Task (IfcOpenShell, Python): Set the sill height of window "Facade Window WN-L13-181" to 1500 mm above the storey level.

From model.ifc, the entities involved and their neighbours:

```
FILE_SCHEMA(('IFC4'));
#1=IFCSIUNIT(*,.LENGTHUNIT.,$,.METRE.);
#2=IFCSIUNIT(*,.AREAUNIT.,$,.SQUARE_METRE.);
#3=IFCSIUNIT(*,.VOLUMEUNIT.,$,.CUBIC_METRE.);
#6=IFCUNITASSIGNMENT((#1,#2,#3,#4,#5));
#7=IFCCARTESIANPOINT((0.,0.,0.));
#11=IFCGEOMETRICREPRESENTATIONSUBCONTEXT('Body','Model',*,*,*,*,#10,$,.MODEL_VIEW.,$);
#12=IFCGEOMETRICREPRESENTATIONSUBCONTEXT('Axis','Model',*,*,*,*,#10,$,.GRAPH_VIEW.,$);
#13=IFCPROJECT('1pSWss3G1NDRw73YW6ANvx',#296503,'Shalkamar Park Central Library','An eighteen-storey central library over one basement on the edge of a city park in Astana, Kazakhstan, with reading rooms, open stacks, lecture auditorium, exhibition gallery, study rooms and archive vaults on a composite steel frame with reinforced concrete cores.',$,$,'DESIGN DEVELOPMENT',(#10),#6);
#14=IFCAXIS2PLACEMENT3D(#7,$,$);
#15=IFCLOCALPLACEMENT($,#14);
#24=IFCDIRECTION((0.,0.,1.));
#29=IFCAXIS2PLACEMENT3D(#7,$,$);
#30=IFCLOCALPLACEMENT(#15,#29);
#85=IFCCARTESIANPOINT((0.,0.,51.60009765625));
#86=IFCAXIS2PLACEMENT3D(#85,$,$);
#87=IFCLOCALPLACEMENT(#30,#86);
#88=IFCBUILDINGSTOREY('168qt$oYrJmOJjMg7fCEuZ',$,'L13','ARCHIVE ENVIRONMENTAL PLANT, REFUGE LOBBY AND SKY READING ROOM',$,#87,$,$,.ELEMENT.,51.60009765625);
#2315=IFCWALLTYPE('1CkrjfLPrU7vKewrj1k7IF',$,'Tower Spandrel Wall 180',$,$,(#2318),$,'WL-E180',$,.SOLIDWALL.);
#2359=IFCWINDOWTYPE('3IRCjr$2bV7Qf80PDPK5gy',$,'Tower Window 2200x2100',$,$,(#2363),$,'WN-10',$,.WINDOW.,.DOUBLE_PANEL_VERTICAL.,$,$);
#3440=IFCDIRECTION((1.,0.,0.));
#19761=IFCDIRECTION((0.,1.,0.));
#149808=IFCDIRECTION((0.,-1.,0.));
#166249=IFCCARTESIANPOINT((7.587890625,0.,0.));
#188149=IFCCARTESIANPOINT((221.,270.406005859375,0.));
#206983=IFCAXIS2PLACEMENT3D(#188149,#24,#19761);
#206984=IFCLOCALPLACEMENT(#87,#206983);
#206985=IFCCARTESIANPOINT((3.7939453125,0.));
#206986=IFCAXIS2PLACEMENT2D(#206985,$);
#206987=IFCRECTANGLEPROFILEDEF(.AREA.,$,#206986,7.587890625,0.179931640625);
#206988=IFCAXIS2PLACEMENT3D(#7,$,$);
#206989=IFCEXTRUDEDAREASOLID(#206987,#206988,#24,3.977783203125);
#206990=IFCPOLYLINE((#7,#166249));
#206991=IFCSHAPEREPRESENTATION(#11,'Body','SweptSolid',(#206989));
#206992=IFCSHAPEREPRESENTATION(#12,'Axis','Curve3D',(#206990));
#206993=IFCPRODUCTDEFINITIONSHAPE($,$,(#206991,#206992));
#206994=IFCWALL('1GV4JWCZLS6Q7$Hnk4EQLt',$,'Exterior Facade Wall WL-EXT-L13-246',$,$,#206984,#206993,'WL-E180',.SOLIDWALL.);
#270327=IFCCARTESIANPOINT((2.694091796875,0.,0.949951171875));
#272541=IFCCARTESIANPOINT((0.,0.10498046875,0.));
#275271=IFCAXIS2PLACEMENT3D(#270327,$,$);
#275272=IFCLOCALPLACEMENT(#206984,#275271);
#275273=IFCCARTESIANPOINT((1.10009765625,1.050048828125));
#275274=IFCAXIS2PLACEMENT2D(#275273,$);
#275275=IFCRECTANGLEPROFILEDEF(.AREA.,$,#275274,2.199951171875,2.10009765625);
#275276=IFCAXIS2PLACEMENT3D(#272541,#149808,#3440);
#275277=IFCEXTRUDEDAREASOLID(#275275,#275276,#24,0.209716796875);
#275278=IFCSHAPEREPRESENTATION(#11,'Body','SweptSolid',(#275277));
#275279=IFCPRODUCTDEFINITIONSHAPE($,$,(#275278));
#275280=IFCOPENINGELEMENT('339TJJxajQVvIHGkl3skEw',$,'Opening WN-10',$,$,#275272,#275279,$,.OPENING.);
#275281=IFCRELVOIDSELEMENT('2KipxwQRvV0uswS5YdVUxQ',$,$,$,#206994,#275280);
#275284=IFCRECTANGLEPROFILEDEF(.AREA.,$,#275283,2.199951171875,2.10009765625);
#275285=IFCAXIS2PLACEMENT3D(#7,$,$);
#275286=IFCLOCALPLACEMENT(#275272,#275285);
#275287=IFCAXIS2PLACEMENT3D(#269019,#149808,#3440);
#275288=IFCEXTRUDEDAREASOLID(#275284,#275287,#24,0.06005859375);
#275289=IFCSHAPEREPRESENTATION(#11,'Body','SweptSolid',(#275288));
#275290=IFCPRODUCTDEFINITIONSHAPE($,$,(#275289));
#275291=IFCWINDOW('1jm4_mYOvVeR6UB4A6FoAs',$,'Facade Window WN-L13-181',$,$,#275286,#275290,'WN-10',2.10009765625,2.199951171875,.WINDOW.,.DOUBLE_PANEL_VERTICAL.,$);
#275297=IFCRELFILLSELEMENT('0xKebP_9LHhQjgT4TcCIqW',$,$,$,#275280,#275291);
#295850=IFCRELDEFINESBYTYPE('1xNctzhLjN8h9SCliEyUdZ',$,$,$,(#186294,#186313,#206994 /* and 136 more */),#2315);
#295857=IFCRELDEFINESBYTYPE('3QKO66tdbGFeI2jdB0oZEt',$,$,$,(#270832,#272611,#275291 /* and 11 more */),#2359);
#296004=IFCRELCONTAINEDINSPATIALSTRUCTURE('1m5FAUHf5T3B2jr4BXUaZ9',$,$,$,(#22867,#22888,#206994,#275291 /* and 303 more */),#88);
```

```python
import numpy as np
import ifcopenshell
import ifcopenshell.api.geometry
import ifcopenshell.geom
import ifcopenshell.util.element
import ifcopenshell.util.placement
import ifcopenshell.util.shape
import ifcopenshell.util.unit

model = ifcopenshell.open("model.ifc")
unit_scale = ifcopenshell.util.unit.calculate_unit_scale(model)

window = model.by_guid("1jm4_mYOvVeR6UB4A6FoAs")
opening = window.FillsVoids[0].RelatingOpeningElement
storey = ifcopenshell.util.element.get_container(window, ifc_class="IfcBuildingStorey")
level = ifcopenshell.util.placement.get_local_placement(storey.ObjectPlacement)[2, 3]

# The opening's origin need not be at the sill, so measure its lowest point.
shape = ifcopenshell.geom.create_shape(ifcopenshell.geom.settings(), opening)
bottom = ifcopenshell.util.shape.get_shape_bottom_elevation(shape, shape.geometry) / unit_scale
dz = level + 1.5 - bottom

shift = np.array([0.0, 0.0, dz])
# The window is placed relative to its opening, so it follows when the opening moves.
matrix = ifcopenshell.util.placement.get_local_placement(opening.ObjectPlacement)
matrix[:3, 3] += shift
ifcopenshell.api.geometry.edit_object_placement(
    model, product=opening, matrix=matrix, is_si=False, should_transform_children=True
)

print(f"moved by {dz * unit_scale:+.3f} m")

model.write("model_rev.ifc")
```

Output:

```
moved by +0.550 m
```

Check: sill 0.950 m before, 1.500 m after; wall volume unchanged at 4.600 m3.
